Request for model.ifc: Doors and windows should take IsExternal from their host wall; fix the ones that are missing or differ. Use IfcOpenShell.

First a look at what the model holds.

```python
import ifcopenshell
import ifcopenshell.util.element

model = ifcopenshell.open("model.ifc")
print(model.schema)
seen = {}
for e in model.by_type("IfcDoor") + model.by_type("IfcWindow"):
    if not e.FillsVoids:
        continue
    host = e.FillsVoids[0].RelatingOpeningElement.VoidsElements[0].RelatingBuildingElement
    own = ifcopenshell.util.element.get_pset(e, f"Pset_{e.is_a()[3:].removesuffix('StandardCase')}Common", "IsExternal")
    wall = ifcopenshell.util.element.get_pset(host, "Pset_WallCommon", "IsExternal")
    seen[e.is_a(), own, wall] = seen.get((e.is_a(), own, wall), 0) + 1
for (cls, own, wall), count in sorted(seen.items(), key=str):
    print(count, cls, "IsExternal:", own, "| host wall:", wall)
```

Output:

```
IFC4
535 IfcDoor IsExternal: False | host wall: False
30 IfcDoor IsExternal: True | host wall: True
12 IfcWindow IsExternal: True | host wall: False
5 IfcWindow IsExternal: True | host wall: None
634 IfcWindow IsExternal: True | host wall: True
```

```python
import ifcopenshell
import ifcopenshell.api.pset
import ifcopenshell.util.element

model = ifcopenshell.open("model.ifc")

count = 0
for ifc_class, pset_name in (("IfcDoor", "Pset_DoorCommon"), ("IfcWindow", "Pset_WindowCommon")):
    for e in model.by_type(ifc_class):
        if not e.FillsVoids:
            continue
        host = e.FillsVoids[0].RelatingOpeningElement.VoidsElements[0].RelatingBuildingElement
        external = ifcopenshell.util.element.get_pset(host, "Pset_WallCommon", "IsExternal")
        if external is None or ifcopenshell.util.element.get_pset(e, pset_name, "IsExternal") == external:
            continue
        pset = ifcopenshell.api.pset.add_pset(model, product=e, name=pset_name)
        ifcopenshell.api.pset.edit_pset(model, pset=pset, properties={"IsExternal": external})
        count += 1

print(count, "updated")

model.write("model_rev.ifc")
```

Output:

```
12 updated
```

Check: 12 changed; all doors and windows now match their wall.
